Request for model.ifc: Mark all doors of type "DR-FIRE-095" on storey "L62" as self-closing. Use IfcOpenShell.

First a look at what the model holds.

```python
import ifcopenshell
import ifcopenshell.util.element

model = ifcopenshell.open("model.ifc")
print(model.schema)
storey = next(s for s in model.by_type("IfcBuildingStorey") if s.Name == "L62")
doors = [e for e in ifcopenshell.util.element.get_decomposition(storey) if e.is_a("IfcDoor")]
seen = {}
for e in doors:
    element_type = ifcopenshell.util.element.get_type(e)
    key = (element_type.Name if element_type != e and element_type else None, ifcopenshell.util.element.get_pset(e, "Pset_DoorCommon", "SelfClosing"))
    seen[key] = seen.get(key, 0) + 1
for (name, value), count in sorted(seen.items(), key=str):
    print(count, "x", name, "|", value)
```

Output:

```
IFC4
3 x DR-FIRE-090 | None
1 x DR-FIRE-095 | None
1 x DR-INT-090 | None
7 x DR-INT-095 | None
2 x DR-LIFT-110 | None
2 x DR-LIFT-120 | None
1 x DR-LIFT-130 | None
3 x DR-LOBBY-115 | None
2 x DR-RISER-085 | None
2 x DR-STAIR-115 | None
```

```python
import ifcopenshell
import ifcopenshell.api.pset
import ifcopenshell.util.element

model = ifcopenshell.open("model.ifc")

storey = next(s for s in model.by_type("IfcBuildingStorey") if s.Name == "L62")
doors = [e for e in ifcopenshell.util.element.get_decomposition(storey) if e.is_a("IfcDoor")]

count = 0
for e in doors:
    element_type = ifcopenshell.util.element.get_type(e)
    if element_type in (None, e) or element_type.Name != "DR-FIRE-095":
        continue
    found = ifcopenshell.util.element.get_pset(e, "Pset_DoorCommon", should_inherit=False)
    if found:
        pset = model.by_id(found["id"])
        if len(ifcopenshell.util.element.get_elements_by_pset(pset)) > 1:
            pset = ifcopenshell.api.pset.unshare_pset(model, products=[e], pset=pset)[0]
    else:
        pset = ifcopenshell.api.pset.add_pset(model, product=e, name="Pset_DoorCommon")
    ifcopenshell.api.pset.edit_pset(model, pset=pset, properties={"SelfClosing": True})
    count += 1

print(count, "doors updated")

model.write("model_v2.ifc")
```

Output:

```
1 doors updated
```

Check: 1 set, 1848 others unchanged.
